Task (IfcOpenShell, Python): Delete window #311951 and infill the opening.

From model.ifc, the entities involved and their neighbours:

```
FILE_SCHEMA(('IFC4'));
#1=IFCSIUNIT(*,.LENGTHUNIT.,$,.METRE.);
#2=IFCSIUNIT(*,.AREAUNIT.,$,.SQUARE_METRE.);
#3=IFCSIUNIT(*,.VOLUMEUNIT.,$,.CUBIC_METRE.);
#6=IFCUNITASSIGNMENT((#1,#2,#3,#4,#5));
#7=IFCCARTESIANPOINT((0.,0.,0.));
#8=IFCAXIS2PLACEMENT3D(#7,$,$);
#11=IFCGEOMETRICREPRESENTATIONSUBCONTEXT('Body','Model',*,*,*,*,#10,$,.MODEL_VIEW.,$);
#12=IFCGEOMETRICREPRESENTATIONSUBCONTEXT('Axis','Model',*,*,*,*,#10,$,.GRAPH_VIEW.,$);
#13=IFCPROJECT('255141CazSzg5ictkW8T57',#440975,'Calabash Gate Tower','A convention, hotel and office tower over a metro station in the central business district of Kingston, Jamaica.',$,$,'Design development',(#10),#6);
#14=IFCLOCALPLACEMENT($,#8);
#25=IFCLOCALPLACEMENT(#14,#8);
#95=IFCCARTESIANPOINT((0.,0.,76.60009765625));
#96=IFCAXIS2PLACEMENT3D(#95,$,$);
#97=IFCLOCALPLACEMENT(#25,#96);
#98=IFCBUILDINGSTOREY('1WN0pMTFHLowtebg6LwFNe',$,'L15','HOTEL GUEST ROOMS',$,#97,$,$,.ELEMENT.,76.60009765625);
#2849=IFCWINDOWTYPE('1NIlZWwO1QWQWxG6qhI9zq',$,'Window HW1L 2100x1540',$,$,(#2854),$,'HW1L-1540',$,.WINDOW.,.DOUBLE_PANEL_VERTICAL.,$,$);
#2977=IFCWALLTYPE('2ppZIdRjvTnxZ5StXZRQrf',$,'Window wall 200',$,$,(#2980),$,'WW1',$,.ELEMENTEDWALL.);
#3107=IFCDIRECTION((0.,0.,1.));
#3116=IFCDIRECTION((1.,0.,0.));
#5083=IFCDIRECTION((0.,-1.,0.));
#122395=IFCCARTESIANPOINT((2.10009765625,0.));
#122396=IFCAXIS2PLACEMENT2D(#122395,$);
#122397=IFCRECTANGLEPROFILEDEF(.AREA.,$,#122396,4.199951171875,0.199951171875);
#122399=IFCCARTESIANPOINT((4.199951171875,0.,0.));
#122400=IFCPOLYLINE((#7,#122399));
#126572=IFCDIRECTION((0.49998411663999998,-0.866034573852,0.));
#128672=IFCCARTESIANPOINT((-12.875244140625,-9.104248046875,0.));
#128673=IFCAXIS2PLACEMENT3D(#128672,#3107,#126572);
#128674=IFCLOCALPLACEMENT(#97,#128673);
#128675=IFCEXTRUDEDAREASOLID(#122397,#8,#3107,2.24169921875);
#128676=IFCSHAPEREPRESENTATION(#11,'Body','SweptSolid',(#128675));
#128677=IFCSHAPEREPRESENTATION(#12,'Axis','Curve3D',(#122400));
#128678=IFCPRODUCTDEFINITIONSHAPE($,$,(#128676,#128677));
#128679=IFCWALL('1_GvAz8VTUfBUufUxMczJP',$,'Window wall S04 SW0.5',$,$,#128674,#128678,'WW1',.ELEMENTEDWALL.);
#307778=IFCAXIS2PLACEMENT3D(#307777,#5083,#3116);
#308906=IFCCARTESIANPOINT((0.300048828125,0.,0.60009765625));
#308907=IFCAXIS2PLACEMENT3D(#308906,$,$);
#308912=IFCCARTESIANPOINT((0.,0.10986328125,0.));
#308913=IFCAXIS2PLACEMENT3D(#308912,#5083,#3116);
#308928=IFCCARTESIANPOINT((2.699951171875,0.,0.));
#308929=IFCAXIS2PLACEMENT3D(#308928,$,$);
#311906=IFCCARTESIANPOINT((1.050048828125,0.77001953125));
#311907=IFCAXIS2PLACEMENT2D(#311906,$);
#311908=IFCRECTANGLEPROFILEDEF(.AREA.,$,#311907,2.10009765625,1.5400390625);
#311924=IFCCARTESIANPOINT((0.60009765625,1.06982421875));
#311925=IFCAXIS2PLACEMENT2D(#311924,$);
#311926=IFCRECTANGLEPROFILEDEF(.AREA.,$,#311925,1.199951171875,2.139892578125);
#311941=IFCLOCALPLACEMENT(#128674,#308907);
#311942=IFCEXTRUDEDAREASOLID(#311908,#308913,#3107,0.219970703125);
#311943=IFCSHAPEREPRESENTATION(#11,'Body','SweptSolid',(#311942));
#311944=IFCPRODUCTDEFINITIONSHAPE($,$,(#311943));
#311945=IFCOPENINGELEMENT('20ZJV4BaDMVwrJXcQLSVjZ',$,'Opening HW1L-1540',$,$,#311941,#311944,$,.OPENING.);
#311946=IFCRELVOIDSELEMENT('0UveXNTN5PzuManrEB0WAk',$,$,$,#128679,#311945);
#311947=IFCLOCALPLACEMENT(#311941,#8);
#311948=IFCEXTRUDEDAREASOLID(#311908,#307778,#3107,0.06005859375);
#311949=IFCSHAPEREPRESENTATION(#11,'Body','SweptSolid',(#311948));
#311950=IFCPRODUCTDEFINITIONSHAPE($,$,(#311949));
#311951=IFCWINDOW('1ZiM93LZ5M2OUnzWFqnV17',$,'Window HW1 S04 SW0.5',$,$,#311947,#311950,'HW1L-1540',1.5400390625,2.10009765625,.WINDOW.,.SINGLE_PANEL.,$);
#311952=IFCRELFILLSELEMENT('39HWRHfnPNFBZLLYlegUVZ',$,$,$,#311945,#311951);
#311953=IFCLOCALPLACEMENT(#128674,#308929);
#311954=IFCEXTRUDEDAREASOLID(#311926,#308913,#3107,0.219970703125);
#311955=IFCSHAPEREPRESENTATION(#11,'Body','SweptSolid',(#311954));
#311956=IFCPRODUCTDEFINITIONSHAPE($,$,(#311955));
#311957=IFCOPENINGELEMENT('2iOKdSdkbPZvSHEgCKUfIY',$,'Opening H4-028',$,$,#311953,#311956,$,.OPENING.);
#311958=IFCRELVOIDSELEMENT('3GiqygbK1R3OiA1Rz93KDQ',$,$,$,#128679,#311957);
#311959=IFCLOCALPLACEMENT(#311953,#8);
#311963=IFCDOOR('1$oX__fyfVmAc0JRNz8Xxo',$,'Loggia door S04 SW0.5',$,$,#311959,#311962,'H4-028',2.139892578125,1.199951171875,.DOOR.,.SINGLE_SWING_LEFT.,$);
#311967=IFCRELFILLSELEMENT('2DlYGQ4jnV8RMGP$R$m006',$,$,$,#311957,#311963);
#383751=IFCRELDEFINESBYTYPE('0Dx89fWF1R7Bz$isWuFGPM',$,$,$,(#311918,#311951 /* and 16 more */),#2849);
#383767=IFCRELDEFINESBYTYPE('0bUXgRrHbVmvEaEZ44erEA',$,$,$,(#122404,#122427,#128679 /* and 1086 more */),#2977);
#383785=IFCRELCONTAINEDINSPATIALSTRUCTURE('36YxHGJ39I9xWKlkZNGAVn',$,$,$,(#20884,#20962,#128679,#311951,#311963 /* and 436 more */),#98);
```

```python
import ifcopenshell
import ifcopenshell.api.feature
import ifcopenshell.api.root
import ifcopenshell.geom
import ifcopenshell.util.shape

model = ifcopenshell.open("model.ifc")
settings = ifcopenshell.geom.settings()


def volume(element):
    """Net volume in cubic metres, openings subtracted."""
    shape = ifcopenshell.geom.create_shape(settings, element)
    return ifcopenshell.util.shape.get_volume(shape.geometry)


window = model.by_id(311951)
opening = window.FillsVoids[0].RelatingOpeningElement
wall = opening.VoidsElements[0].RelatingBuildingElement
before = volume(wall)

ifcopenshell.api.root.remove_product(model, product=window)
ifcopenshell.api.feature.remove_feature(model, feature=opening)

after = volume(wall)

print(f"wall volume {before:.3f} -> {after:.3f} m3")

model.write("model_updated.ifc")
```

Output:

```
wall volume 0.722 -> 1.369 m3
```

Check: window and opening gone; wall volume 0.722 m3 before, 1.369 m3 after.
